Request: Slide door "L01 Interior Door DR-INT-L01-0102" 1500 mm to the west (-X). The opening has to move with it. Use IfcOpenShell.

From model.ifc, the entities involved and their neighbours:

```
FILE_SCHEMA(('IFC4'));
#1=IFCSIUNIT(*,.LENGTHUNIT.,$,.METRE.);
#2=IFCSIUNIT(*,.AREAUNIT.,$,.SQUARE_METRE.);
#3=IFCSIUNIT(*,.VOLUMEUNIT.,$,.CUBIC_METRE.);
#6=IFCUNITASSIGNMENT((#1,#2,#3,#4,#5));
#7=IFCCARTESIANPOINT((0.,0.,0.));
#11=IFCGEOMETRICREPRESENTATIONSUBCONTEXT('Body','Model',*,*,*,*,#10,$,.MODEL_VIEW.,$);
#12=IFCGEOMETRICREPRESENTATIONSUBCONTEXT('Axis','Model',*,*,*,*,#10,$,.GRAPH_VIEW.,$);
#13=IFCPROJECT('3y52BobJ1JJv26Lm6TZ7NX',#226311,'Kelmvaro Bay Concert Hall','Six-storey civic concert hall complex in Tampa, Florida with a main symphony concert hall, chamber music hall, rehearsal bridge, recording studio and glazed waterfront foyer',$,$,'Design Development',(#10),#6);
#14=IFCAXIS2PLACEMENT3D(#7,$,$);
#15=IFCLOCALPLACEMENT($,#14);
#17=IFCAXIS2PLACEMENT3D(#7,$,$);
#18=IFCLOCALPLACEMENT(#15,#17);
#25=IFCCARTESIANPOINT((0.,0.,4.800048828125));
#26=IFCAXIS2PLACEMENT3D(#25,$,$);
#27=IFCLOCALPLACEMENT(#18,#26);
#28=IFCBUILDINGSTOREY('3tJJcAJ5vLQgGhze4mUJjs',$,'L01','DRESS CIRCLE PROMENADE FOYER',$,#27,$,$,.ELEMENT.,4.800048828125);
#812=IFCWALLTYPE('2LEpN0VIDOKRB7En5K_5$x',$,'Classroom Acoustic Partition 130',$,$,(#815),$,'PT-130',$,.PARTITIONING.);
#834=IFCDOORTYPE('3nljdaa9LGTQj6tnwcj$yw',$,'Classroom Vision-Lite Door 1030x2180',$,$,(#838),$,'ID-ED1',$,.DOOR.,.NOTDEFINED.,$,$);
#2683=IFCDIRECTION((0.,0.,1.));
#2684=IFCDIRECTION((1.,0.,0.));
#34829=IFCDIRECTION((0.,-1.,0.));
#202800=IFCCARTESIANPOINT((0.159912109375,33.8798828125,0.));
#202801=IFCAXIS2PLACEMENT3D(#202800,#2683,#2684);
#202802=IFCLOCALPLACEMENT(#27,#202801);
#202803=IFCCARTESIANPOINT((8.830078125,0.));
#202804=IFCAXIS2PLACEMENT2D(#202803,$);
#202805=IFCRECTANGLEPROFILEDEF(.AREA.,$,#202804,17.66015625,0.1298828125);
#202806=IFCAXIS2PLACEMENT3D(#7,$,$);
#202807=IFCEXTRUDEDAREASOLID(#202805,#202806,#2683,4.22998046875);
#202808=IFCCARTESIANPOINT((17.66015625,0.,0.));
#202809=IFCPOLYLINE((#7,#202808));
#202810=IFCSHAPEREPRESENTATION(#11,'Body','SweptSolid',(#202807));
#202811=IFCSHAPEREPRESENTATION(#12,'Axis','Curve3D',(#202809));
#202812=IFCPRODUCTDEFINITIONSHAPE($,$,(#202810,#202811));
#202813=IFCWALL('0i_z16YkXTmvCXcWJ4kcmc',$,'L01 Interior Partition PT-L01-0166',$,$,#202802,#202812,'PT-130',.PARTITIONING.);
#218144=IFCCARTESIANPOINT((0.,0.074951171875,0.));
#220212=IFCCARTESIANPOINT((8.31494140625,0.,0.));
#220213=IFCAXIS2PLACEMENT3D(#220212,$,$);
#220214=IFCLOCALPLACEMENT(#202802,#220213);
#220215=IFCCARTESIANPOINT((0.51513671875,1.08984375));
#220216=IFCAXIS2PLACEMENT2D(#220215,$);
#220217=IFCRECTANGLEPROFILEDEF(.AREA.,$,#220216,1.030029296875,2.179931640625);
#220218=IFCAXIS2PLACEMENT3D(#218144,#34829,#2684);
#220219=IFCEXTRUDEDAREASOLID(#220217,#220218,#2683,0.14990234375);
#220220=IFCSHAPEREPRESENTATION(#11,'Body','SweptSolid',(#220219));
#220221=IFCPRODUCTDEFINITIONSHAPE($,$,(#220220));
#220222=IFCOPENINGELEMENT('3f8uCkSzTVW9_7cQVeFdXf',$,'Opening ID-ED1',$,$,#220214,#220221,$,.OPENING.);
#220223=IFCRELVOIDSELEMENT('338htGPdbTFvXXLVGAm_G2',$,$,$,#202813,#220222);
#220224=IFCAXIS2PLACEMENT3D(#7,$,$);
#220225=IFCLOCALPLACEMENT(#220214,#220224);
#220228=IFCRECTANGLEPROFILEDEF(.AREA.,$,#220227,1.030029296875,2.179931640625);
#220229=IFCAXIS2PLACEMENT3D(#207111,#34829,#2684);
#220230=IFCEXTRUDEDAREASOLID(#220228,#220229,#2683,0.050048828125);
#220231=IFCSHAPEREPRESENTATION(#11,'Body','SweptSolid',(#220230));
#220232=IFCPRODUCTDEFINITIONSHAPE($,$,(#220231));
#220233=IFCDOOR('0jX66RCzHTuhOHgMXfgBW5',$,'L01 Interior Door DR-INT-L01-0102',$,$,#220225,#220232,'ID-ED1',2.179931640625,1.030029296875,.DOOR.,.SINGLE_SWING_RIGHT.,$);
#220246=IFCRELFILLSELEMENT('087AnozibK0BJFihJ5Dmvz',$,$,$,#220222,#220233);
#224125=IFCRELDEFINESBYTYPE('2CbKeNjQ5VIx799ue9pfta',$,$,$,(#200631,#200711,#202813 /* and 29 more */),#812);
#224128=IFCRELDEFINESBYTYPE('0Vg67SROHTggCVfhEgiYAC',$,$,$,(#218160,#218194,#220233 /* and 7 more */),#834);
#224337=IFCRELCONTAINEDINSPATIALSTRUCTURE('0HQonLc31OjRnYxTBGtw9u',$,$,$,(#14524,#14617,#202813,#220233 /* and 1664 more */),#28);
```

```python
import ifcopenshell
import ifcopenshell.api.geometry
import ifcopenshell.util.placement

model = ifcopenshell.open("model.ifc")

door = model.by_guid("0jX66RCzHTuhOHgMXfgBW5")
opening = door.FillsVoids[0].RelatingOpeningElement
wall = opening.VoidsElements[0].RelatingBuildingElement

wall_matrix = ifcopenshell.util.placement.get_local_placement(wall.ObjectPlacement)
shift = wall_matrix[:3, 0] * -1.5
before = ifcopenshell.util.placement.get_local_placement(door.ObjectPlacement)[:3, 3].copy()

# The door is placed relative to its opening, so it follows when the opening moves.
matrix = ifcopenshell.util.placement.get_local_placement(opening.ObjectPlacement)
matrix[:3, 3] += shift
ifcopenshell.api.geometry.edit_object_placement(
    model, product=opening, matrix=matrix, is_si=False, should_transform_children=True
)

after = ifcopenshell.util.placement.get_local_placement(door.ObjectPlacement)[:3, 3]
print("door moved by", (after - before).round(3) + 0.0)

model.write("model-out.ifc")
```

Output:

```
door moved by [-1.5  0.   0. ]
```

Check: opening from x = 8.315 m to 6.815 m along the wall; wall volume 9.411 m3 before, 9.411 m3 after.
